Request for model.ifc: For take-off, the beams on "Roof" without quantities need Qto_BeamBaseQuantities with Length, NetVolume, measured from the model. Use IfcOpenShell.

First a look at what the model holds.

```python
import ifcopenshell
import ifcopenshell.util.element
import ifcopenshell.util.unit

model = ifcopenshell.open("model.ifc")
print(model.schema)
for unit_type in ("LENGTHUNIT", "AREAUNIT", "VOLUMEUNIT"):
    print(unit_type, ifcopenshell.util.unit.calculate_unit_scale(model, unit_type))
storey = next(s for s in model.by_type("IfcBuildingStorey") if s.Name == "Roof")
beams = [e for e in ifcopenshell.util.element.get_decomposition(storey) if e.is_a("IfcBeam")]
for e in sorted(beams, key=lambda e: e.id()):
    print(e.id(), e.is_a(), e.Name, list(ifcopenshell.util.element.get_psets(e, qtos_only=True)), sep=" | ")
```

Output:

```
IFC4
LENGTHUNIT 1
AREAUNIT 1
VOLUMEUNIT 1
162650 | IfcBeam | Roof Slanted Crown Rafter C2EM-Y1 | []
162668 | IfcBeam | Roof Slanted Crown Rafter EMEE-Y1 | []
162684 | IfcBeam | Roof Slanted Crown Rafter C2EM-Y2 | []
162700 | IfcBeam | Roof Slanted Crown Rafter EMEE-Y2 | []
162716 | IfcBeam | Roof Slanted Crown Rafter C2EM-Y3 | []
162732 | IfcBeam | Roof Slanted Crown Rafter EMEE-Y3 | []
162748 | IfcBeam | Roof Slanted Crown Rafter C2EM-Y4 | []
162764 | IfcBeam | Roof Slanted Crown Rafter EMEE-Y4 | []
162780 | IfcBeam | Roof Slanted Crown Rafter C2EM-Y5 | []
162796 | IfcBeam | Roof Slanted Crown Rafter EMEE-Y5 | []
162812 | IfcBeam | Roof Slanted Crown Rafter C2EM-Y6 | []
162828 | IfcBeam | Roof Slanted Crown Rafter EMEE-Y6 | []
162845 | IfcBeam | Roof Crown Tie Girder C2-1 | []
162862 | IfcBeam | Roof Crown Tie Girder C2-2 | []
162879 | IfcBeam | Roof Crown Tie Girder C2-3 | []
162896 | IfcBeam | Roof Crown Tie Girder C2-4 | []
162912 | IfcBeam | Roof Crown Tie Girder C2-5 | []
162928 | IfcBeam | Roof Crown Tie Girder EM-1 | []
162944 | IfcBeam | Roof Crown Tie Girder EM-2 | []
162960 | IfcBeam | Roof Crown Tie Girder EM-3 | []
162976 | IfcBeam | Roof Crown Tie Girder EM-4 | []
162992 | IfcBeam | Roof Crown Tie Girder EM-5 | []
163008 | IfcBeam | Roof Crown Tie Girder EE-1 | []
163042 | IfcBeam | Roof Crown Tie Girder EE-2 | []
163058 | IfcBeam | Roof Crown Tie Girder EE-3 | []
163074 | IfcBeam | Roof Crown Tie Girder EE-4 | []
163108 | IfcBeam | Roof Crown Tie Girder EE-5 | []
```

```python
import ifcopenshell
import ifcopenshell.api.pset
import ifcopenshell.geom
import ifcopenshell.util.element
import ifcopenshell.util.shape
import ifcopenshell.util.unit

model = ifcopenshell.open("model.ifc")
unit_scale = ifcopenshell.util.unit.calculate_unit_scale(model)
volume_scale = ifcopenshell.util.unit.calculate_unit_scale(model, "VOLUMEUNIT")
settings = ifcopenshell.geom.settings()

storey = next(s for s in model.by_type("IfcBuildingStorey") if s.Name == "Roof")
beams = [e for e in ifcopenshell.util.element.get_decomposition(storey) if e.is_a("IfcBeam")]

for e in sorted(beams, key=lambda e: e.id()):
    if ifcopenshell.util.element.get_psets(e, qtos_only=True, should_inherit=False):
        continue
    # Geometry comes back in metres, in the element's own axes.
    shape = ifcopenshell.geom.create_shape(settings, e)
    values = {
        "Length": ifcopenshell.util.shape.get_max_xyz(shape.geometry) / unit_scale,
        "NetVolume": ifcopenshell.util.shape.get_volume(shape.geometry) / volume_scale,
    }
    qto = ifcopenshell.api.pset.add_qto(model, product=e, name="Qto_BeamBaseQuantities")
    ifcopenshell.api.pset.edit_qto(model, qto=qto, properties=values)
    print(e.id(), {k: round(v, 3) for k, v in values.items()})

model.write("model_v2.ifc")
```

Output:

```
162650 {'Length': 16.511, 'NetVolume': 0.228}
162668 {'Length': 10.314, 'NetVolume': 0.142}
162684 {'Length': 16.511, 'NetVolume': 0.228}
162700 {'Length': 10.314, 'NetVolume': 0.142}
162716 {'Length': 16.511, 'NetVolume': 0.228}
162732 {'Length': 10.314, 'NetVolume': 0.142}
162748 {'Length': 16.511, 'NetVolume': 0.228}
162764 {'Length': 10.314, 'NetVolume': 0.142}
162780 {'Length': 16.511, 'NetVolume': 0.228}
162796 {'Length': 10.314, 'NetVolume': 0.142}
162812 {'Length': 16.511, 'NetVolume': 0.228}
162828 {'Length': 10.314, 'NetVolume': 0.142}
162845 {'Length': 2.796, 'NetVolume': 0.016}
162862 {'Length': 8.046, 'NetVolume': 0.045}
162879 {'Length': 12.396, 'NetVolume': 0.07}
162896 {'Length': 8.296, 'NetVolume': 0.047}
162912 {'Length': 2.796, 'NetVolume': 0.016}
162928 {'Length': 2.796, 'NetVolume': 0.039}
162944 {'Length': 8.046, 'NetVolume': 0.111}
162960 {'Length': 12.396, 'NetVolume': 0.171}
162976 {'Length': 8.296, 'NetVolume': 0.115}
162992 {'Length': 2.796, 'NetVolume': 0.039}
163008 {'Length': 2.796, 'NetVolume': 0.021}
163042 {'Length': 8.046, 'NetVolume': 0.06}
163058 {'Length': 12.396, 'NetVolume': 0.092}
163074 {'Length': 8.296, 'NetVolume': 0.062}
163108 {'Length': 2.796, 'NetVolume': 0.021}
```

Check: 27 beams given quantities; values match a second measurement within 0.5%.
